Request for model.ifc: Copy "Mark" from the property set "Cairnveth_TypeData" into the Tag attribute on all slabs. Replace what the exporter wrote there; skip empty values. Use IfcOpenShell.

First a look at what the model holds.

```python
import ifcopenshell
import ifcopenshell.util.element

model = ifcopenshell.open("model.ifc")
print(model.schema)
slabs = model.by_type("IfcSlab")
print(len(slabs), "slabs")
for e in slabs[:8]:
    source = ifcopenshell.util.element.get_pset(e, "Cairnveth_TypeData", "Mark")
    target = e.Tag
    print(e.id(), repr(source), repr(target), sep=" | ")
```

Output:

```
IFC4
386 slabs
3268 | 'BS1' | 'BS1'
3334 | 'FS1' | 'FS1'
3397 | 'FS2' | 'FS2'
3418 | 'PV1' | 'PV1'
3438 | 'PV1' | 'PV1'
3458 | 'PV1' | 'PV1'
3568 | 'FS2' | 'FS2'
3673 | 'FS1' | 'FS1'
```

```python
import ifcopenshell
import ifcopenshell.util.element

model = ifcopenshell.open("model.ifc")

count = 0
for e in model.by_type("IfcSlab"):
    value = ifcopenshell.util.element.get_pset(e, "Cairnveth_TypeData", "Mark")
    current = e.Tag
    if not value or not value.strip() or current == value:
        continue
    e.Tag = value
    count += 1

print(count, "slabs updated")

model.write("model_rev.ifc")
```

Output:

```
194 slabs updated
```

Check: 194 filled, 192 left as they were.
